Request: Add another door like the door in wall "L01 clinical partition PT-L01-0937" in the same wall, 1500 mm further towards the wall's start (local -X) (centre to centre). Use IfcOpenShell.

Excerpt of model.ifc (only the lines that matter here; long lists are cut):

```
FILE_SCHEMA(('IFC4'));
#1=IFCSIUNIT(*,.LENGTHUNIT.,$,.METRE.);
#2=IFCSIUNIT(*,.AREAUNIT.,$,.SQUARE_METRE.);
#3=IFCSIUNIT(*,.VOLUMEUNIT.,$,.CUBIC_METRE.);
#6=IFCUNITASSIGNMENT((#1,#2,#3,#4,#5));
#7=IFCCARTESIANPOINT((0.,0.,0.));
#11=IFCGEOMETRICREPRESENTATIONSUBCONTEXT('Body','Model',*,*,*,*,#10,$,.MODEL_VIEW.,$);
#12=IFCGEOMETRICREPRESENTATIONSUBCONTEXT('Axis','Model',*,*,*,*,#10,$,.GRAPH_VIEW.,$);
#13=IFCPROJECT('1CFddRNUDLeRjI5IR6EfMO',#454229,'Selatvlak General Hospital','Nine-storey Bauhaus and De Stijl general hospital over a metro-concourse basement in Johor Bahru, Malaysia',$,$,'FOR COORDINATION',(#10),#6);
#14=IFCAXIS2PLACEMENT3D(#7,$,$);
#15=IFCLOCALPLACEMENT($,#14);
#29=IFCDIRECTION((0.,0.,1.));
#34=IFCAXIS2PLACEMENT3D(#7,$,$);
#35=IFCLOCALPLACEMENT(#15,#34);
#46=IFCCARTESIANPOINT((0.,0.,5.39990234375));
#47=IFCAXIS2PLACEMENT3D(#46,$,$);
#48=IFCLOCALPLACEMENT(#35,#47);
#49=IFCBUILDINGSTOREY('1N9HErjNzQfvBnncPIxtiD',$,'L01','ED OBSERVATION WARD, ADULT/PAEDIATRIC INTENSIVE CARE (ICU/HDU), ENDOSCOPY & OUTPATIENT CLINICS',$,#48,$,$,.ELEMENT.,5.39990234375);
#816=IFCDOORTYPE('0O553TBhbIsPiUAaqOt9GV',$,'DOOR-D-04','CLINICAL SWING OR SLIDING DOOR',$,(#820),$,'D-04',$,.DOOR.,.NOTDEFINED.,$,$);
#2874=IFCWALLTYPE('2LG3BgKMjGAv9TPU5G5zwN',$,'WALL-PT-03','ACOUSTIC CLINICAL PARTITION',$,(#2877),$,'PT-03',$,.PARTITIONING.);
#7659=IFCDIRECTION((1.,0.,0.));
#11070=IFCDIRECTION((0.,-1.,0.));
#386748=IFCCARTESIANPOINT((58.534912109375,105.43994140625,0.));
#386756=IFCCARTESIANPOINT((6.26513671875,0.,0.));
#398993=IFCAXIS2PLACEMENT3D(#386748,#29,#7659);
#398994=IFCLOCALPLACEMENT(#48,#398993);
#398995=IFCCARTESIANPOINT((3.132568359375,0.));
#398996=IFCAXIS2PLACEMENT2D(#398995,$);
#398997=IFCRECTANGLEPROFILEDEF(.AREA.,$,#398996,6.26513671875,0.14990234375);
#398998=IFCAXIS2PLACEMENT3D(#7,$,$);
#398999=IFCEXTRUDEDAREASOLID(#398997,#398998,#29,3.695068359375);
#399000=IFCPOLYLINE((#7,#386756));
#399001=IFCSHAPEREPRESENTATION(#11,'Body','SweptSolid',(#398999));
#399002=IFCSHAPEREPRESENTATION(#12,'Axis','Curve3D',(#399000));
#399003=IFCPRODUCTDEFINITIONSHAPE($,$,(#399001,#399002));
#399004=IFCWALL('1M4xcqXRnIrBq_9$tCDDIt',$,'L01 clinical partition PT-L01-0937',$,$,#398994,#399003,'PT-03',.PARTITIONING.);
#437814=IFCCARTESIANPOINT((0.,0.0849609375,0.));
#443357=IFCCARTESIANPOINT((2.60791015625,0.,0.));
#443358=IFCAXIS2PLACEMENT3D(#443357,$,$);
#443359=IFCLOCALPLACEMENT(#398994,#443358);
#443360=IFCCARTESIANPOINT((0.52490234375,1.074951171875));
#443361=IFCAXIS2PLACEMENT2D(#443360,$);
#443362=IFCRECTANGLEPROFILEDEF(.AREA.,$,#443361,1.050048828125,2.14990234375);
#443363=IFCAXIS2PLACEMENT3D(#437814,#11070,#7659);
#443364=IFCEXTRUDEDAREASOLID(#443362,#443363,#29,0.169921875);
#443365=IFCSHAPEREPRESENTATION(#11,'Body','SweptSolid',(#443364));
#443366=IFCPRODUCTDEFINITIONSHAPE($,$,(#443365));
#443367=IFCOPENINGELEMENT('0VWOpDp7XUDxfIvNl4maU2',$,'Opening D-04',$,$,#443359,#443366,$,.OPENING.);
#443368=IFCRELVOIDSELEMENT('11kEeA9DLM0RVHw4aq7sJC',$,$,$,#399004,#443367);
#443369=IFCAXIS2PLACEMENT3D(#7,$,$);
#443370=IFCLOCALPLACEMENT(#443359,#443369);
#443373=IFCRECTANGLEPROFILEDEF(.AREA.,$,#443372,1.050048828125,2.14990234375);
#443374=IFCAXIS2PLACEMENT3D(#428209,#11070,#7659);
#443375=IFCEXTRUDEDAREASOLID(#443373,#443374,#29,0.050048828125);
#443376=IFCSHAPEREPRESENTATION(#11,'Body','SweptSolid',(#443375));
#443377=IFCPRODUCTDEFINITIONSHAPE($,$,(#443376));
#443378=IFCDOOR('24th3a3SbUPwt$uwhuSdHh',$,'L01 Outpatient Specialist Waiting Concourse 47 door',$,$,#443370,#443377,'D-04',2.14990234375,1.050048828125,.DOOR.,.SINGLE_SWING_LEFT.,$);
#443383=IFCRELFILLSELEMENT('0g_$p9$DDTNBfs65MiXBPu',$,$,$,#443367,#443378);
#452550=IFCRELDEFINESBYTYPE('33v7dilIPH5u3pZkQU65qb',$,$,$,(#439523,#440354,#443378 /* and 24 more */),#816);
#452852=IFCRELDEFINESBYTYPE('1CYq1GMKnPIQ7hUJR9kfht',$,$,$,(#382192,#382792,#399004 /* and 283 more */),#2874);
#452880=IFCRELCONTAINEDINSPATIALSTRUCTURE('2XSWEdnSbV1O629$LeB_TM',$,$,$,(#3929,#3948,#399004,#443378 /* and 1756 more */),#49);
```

```python
import ifcopenshell
import ifcopenshell.api.feature
import ifcopenshell.api.geometry
import ifcopenshell.api.root
import ifcopenshell.geom
import ifcopenshell.util.element
import ifcopenshell.util.placement
import ifcopenshell.util.shape

model = ifcopenshell.open("model.ifc")
settings = ifcopenshell.geom.settings()


def volume(element):
    """Net volume in cubic metres, openings subtracted."""
    shape = ifcopenshell.geom.create_shape(settings, element)
    return ifcopenshell.util.shape.get_volume(shape.geometry)


door = model.by_id(443378)
opening = door.FillsVoids[0].RelatingOpeningElement
wall = opening.VoidsElements[0].RelatingBuildingElement
before = volume(wall)
shift = ifcopenshell.util.placement.get_local_placement(wall.ObjectPlacement)[:3, 0] * -1.5

# copy_class copies the void relationship, type, container and properties, but no geometry.
new_opening = ifcopenshell.api.root.copy_class(model, product=opening)
new_opening.Representation = ifcopenshell.util.element.copy_deep(
    model, opening.Representation, exclude=["IfcGeometricRepresentationContext", "IfcRepresentationMap"]
)
new_door = ifcopenshell.api.root.copy_class(model, product=door)
new_door.Representation = ifcopenshell.util.element.copy_deep(
    model, door.Representation, exclude=["IfcGeometricRepresentationContext", "IfcRepresentationMap"]
)
new_door.Tag = None
ifcopenshell.api.feature.add_filling(model, opening=new_opening, element=new_door)

for old, new in ((opening, new_opening), (door, new_door)):
    matrix = ifcopenshell.util.placement.get_local_placement(old.ObjectPlacement)
    matrix[:3, 3] += shift
    ifcopenshell.api.geometry.edit_object_placement(model, product=new, matrix=matrix, is_si=False)

after = volume(wall)

print(f"wall volume {before:.3f} -> {after:.3f} m3")

model.write("model_rev.ifc")
```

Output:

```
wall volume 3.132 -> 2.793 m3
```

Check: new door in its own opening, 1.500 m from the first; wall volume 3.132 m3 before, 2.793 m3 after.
